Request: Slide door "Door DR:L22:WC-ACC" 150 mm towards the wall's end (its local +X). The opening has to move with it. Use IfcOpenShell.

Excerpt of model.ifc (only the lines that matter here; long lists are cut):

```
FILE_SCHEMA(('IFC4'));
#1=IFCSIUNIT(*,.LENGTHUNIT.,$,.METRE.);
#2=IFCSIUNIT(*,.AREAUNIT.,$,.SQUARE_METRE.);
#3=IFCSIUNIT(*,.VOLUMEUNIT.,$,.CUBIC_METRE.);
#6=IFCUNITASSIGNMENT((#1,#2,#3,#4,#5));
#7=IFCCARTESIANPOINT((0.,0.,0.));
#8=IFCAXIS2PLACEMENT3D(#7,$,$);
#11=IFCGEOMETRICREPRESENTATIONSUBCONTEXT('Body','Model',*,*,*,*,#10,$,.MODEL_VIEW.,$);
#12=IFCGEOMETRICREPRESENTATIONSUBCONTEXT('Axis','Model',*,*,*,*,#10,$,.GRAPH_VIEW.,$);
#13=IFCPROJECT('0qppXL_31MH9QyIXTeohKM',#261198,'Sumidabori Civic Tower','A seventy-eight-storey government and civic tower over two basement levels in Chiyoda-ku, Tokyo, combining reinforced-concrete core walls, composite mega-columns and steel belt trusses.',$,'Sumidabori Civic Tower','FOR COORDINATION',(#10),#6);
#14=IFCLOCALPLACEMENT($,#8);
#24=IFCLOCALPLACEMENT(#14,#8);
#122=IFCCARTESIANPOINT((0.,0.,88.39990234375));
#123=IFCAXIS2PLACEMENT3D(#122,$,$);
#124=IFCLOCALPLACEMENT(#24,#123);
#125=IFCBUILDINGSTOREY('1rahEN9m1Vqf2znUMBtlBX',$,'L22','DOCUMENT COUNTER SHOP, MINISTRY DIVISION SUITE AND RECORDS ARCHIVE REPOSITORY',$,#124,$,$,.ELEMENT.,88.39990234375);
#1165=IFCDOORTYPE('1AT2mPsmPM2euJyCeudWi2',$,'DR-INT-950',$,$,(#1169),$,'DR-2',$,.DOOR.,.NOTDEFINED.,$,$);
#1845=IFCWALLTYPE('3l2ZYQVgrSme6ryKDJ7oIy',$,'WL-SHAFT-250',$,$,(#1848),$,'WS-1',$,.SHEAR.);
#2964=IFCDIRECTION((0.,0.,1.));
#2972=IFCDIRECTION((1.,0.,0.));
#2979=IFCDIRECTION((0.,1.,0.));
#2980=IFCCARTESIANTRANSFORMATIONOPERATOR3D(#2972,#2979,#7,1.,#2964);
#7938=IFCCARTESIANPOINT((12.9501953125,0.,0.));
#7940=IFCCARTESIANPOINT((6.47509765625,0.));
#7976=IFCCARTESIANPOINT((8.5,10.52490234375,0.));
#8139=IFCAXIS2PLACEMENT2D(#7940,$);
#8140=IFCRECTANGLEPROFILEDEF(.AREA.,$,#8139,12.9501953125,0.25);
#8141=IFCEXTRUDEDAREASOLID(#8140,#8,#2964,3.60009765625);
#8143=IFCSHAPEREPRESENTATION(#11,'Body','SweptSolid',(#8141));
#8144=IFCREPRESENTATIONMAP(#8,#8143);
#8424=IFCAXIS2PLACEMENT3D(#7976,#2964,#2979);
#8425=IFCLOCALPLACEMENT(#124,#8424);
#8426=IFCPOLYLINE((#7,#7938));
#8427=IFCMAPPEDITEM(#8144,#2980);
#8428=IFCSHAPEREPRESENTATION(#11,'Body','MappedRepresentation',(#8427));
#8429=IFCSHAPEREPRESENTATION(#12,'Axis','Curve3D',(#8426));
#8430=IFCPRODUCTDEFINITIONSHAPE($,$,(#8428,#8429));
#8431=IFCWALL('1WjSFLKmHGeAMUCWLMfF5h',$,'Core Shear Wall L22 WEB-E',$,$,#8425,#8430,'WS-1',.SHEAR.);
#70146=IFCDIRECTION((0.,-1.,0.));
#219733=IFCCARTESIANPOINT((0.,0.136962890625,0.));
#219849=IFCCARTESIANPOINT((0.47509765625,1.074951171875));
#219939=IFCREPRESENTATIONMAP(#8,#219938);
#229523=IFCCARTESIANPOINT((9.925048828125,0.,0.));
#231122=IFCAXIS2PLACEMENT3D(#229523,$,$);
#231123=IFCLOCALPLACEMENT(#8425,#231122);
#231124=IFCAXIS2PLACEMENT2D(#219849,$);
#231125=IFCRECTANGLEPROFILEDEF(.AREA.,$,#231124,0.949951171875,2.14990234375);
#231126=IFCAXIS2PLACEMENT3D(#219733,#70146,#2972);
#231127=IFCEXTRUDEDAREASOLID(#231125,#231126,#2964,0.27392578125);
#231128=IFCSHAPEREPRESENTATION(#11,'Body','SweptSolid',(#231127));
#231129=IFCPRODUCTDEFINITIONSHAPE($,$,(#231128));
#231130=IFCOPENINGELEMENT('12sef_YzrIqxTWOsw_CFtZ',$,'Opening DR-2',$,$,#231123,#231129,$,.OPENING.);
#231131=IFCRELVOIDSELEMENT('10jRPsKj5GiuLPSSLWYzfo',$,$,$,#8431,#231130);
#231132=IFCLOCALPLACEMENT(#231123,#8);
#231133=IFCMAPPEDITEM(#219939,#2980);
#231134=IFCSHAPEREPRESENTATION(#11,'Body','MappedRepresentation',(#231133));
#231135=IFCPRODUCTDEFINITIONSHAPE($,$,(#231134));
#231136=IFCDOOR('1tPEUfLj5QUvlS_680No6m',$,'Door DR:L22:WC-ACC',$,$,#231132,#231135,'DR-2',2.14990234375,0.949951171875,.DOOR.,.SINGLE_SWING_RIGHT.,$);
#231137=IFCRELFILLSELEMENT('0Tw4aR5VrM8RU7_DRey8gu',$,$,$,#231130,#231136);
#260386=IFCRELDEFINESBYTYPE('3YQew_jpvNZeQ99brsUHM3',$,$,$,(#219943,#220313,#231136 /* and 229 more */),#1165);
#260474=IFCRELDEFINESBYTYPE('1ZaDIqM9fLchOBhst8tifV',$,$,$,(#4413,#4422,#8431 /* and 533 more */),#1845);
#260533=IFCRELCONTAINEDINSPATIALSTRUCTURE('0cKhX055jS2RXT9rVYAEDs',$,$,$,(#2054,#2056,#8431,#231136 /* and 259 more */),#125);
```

```python
import ifcopenshell
import ifcopenshell.api.geometry
import ifcopenshell.util.placement
import ifcopenshell.util.unit

model = ifcopenshell.open("model.ifc")
unit_scale = ifcopenshell.util.unit.calculate_unit_scale(model)

door = model.by_guid("1tPEUfLj5QUvlS_680No6m")
opening = door.FillsVoids[0].RelatingOpeningElement
wall = opening.VoidsElements[0].RelatingBuildingElement

wall_matrix = ifcopenshell.util.placement.get_local_placement(wall.ObjectPlacement)
shift = wall_matrix[:3, 0] * 0.15 / unit_scale
before = ifcopenshell.util.placement.get_local_placement(door.ObjectPlacement)[:3, 3].copy()

# The door is placed relative to its opening, so it follows when the opening moves.
matrix = ifcopenshell.util.placement.get_local_placement(opening.ObjectPlacement)
matrix[:3, 3] += shift
ifcopenshell.api.geometry.edit_object_placement(
    model, product=opening, matrix=matrix, is_si=False, should_transform_children=True
)

after = ifcopenshell.util.placement.get_local_placement(door.ObjectPlacement)[:3, 3]
print("door moved by", (after - before).round(3) + 0.0)

model.write("model_rev.ifc")
```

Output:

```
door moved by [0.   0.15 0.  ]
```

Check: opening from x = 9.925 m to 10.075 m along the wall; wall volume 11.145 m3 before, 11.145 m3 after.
